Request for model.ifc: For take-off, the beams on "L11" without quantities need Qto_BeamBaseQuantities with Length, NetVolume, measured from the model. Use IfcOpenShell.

First a look at what the model holds.

```python
import ifcopenshell
import ifcopenshell.util.element
import ifcopenshell.util.unit

model = ifcopenshell.open("model.ifc")
print(model.schema)
for unit_type in ("LENGTHUNIT", "AREAUNIT", "VOLUMEUNIT"):
    print(unit_type, ifcopenshell.util.unit.calculate_unit_scale(model, unit_type))
storey = next(s for s in model.by_type("IfcBuildingStorey") if s.Name == "L11")
beams = [e for e in ifcopenshell.util.element.get_decomposition(storey) if e.is_a("IfcBeam")]
for e in sorted(beams, key=lambda e: e.id()):
    print(e.id(), e.is_a(), e.Name, list(ifcopenshell.util.element.get_psets(e, qtos_only=True)), sep=" | ")
```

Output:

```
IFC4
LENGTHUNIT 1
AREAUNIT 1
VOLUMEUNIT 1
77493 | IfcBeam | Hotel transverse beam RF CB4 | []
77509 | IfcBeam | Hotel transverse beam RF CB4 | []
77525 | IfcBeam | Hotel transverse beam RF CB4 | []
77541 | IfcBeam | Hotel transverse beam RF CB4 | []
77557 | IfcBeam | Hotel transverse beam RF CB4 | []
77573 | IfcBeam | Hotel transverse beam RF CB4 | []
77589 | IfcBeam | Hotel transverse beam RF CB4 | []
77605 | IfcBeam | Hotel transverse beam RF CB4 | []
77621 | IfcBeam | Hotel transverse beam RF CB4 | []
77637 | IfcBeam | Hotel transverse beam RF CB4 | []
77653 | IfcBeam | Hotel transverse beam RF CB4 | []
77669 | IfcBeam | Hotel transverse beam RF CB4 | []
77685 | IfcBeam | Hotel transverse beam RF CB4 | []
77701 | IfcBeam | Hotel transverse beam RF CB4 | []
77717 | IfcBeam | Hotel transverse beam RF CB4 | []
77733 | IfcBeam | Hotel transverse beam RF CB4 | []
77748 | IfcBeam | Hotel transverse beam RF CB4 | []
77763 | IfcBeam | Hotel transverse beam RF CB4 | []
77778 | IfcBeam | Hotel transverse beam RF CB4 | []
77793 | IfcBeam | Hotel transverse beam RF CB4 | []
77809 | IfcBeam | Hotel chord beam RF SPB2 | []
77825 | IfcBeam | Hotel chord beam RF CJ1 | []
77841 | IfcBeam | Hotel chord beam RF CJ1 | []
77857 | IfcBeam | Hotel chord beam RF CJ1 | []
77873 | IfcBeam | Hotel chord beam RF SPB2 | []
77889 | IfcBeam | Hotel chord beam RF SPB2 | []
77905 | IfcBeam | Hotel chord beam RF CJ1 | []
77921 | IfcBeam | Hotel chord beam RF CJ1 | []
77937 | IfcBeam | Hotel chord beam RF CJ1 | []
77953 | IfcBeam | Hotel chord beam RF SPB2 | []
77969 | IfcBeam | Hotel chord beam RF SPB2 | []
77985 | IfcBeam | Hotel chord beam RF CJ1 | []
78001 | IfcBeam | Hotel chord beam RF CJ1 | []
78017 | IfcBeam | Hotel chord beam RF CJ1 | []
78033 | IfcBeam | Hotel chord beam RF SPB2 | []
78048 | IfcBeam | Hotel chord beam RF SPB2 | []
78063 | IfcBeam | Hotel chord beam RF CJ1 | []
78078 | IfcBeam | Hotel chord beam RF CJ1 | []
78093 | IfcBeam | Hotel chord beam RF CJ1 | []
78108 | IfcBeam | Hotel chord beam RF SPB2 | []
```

```python
import ifcopenshell
import ifcopenshell.api.pset
import ifcopenshell.geom
import ifcopenshell.util.element
import ifcopenshell.util.shape
import ifcopenshell.util.unit

model = ifcopenshell.open("model.ifc")
unit_scale = ifcopenshell.util.unit.calculate_unit_scale(model)
volume_scale = ifcopenshell.util.unit.calculate_unit_scale(model, "VOLUMEUNIT")
settings = ifcopenshell.geom.settings()

storey = next(s for s in model.by_type("IfcBuildingStorey") if s.Name == "L11")
beams = [e for e in ifcopenshell.util.element.get_decomposition(storey) if e.is_a("IfcBeam")]

for e in sorted(beams, key=lambda e: e.id()):
    if ifcopenshell.util.element.get_psets(e, qtos_only=True, should_inherit=False):
        continue
    # Geometry comes back in metres, in the element's own axes.
    shape = ifcopenshell.geom.create_shape(settings, e)
    values = {
        "Length": ifcopenshell.util.shape.get_max_xyz(shape.geometry) / unit_scale,
        "NetVolume": ifcopenshell.util.shape.get_volume(shape.geometry) / volume_scale,
    }
    qto = ifcopenshell.api.pset.add_qto(model, product=e, name="Qto_BeamBaseQuantities")
    ifcopenshell.api.pset.edit_qto(model, qto=qto, properties=values)
    print(e.id(), {k: round(v, 3) for k, v in values.items()})

model.write("model_updated.ifc")
```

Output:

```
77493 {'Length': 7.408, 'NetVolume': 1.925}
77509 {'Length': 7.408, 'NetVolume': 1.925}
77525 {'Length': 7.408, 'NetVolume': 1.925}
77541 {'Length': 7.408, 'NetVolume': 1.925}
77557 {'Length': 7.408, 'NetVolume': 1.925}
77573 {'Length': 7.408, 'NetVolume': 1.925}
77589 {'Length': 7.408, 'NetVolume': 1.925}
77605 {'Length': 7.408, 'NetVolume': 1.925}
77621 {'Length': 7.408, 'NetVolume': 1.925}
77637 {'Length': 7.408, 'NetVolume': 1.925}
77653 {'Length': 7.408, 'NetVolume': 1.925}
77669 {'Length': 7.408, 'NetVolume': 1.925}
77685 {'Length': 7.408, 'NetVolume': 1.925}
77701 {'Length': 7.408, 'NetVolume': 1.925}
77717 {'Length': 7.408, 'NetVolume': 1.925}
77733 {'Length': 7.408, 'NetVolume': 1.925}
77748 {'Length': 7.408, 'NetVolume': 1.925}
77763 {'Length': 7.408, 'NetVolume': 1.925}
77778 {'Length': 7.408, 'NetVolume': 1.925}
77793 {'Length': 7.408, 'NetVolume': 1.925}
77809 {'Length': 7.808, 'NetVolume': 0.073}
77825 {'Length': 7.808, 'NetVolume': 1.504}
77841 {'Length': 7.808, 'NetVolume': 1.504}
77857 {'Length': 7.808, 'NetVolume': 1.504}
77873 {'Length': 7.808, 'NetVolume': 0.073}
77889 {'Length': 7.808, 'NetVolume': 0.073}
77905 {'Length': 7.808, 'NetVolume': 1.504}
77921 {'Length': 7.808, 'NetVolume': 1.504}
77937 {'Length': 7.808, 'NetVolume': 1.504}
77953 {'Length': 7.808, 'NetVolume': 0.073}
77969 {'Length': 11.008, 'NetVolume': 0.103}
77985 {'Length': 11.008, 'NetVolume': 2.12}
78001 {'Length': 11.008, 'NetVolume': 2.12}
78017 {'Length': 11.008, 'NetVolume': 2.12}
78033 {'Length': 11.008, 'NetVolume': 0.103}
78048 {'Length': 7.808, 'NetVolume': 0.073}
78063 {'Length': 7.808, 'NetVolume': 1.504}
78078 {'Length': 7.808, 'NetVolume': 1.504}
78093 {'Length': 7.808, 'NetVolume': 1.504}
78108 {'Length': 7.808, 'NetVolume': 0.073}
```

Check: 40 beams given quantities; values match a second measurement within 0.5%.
